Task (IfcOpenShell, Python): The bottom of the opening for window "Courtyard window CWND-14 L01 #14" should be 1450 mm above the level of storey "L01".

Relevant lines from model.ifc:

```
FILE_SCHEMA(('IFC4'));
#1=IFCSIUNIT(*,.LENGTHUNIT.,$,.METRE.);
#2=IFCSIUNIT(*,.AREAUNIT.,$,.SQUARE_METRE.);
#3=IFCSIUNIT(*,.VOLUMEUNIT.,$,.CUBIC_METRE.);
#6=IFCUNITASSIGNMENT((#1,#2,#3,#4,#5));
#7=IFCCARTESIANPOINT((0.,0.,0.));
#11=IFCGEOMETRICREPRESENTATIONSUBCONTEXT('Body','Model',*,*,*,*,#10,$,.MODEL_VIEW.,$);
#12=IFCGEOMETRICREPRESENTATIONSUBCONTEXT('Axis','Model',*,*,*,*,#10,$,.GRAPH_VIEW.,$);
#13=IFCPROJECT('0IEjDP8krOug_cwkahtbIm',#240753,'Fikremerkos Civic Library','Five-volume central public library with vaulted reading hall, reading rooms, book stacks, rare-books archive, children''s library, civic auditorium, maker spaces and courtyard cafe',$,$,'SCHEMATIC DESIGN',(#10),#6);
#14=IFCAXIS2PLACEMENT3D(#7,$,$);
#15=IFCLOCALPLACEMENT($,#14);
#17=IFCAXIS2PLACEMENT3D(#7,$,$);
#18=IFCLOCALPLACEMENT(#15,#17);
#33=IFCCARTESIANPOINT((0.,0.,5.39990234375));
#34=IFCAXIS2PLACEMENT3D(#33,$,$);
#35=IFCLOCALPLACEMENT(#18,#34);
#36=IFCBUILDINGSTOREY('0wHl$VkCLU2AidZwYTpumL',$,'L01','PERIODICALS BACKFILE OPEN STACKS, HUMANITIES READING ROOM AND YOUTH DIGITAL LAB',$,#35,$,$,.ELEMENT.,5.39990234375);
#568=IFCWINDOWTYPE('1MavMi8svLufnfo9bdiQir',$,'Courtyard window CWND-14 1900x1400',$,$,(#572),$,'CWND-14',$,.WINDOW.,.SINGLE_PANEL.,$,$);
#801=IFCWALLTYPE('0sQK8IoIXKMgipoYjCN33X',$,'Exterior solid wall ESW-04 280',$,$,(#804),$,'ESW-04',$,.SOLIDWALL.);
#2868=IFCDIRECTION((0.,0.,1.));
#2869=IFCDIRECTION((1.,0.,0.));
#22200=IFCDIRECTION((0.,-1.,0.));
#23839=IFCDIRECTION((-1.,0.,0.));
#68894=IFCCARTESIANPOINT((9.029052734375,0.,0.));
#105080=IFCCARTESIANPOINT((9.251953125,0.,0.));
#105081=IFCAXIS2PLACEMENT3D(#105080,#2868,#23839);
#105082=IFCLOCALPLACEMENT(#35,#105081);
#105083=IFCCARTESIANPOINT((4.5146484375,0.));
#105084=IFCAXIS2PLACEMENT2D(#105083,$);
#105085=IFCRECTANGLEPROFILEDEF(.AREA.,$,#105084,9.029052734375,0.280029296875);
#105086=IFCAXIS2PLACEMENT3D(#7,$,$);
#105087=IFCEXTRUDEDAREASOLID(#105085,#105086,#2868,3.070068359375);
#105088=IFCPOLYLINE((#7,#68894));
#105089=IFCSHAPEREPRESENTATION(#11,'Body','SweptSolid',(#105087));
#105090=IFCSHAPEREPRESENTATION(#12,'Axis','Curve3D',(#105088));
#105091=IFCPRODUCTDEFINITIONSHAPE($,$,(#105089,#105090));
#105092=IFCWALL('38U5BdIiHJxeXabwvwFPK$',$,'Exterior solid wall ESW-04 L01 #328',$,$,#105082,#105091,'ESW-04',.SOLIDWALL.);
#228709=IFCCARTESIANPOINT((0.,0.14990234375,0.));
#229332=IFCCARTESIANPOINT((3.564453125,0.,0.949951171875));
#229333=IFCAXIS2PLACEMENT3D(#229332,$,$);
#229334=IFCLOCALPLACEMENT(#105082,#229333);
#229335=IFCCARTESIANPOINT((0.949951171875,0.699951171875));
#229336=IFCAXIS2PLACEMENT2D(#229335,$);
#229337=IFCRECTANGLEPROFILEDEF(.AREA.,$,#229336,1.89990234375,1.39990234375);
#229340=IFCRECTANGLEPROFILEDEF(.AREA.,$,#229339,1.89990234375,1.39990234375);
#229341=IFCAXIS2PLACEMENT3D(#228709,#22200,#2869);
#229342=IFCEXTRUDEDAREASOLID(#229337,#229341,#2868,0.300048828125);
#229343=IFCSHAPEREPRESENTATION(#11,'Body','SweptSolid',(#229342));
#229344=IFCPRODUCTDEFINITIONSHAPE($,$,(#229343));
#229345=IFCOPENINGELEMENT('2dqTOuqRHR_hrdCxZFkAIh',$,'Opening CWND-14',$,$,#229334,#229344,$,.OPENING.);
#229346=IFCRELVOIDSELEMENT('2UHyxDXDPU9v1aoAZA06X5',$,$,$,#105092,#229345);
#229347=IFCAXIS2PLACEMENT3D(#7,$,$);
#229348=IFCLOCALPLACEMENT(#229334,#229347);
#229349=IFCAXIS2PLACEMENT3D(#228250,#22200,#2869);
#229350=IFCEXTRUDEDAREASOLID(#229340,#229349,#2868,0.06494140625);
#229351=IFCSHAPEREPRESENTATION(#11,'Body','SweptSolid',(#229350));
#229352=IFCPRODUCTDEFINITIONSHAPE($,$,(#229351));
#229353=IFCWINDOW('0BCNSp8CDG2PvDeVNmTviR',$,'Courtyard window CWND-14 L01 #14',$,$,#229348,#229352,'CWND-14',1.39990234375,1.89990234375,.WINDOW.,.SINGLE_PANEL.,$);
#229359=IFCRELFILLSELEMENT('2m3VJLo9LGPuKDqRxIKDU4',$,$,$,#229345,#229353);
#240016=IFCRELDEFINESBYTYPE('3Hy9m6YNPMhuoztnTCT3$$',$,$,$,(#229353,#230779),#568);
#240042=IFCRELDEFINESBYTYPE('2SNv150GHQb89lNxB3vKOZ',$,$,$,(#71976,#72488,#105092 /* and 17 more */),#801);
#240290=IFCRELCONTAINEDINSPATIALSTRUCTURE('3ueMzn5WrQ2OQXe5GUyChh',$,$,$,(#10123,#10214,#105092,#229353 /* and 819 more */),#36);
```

```python
import numpy as np
import ifcopenshell
import ifcopenshell.api.geometry
import ifcopenshell.geom
import ifcopenshell.util.element
import ifcopenshell.util.placement
import ifcopenshell.util.shape
import ifcopenshell.util.unit

model = ifcopenshell.open("model.ifc")
unit_scale = ifcopenshell.util.unit.calculate_unit_scale(model)

window = model.by_guid("0BCNSp8CDG2PvDeVNmTviR")
opening = window.FillsVoids[0].RelatingOpeningElement
storey = ifcopenshell.util.element.get_container(window, ifc_class="IfcBuildingStorey")
level = ifcopenshell.util.placement.get_local_placement(storey.ObjectPlacement)[2, 3]

# The opening's origin need not be at the sill, so measure its lowest point.
shape = ifcopenshell.geom.create_shape(ifcopenshell.geom.settings(), opening)
bottom = ifcopenshell.util.shape.get_shape_bottom_elevation(shape, shape.geometry) / unit_scale
dz = level + 1.45 - bottom

shift = np.array([0.0, 0.0, dz])
# The window is placed relative to its opening, so it follows when the opening moves.
matrix = ifcopenshell.util.placement.get_local_placement(opening.ObjectPlacement)
matrix[:3, 3] += shift
ifcopenshell.api.geometry.edit_object_placement(
    model, product=opening, matrix=matrix, is_si=False, should_transform_children=True
)

print(f"moved by {dz * unit_scale:+.3f} m")

model.write("model_updated.ifc")
```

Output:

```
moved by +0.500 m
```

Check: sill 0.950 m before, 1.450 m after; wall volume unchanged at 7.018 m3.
